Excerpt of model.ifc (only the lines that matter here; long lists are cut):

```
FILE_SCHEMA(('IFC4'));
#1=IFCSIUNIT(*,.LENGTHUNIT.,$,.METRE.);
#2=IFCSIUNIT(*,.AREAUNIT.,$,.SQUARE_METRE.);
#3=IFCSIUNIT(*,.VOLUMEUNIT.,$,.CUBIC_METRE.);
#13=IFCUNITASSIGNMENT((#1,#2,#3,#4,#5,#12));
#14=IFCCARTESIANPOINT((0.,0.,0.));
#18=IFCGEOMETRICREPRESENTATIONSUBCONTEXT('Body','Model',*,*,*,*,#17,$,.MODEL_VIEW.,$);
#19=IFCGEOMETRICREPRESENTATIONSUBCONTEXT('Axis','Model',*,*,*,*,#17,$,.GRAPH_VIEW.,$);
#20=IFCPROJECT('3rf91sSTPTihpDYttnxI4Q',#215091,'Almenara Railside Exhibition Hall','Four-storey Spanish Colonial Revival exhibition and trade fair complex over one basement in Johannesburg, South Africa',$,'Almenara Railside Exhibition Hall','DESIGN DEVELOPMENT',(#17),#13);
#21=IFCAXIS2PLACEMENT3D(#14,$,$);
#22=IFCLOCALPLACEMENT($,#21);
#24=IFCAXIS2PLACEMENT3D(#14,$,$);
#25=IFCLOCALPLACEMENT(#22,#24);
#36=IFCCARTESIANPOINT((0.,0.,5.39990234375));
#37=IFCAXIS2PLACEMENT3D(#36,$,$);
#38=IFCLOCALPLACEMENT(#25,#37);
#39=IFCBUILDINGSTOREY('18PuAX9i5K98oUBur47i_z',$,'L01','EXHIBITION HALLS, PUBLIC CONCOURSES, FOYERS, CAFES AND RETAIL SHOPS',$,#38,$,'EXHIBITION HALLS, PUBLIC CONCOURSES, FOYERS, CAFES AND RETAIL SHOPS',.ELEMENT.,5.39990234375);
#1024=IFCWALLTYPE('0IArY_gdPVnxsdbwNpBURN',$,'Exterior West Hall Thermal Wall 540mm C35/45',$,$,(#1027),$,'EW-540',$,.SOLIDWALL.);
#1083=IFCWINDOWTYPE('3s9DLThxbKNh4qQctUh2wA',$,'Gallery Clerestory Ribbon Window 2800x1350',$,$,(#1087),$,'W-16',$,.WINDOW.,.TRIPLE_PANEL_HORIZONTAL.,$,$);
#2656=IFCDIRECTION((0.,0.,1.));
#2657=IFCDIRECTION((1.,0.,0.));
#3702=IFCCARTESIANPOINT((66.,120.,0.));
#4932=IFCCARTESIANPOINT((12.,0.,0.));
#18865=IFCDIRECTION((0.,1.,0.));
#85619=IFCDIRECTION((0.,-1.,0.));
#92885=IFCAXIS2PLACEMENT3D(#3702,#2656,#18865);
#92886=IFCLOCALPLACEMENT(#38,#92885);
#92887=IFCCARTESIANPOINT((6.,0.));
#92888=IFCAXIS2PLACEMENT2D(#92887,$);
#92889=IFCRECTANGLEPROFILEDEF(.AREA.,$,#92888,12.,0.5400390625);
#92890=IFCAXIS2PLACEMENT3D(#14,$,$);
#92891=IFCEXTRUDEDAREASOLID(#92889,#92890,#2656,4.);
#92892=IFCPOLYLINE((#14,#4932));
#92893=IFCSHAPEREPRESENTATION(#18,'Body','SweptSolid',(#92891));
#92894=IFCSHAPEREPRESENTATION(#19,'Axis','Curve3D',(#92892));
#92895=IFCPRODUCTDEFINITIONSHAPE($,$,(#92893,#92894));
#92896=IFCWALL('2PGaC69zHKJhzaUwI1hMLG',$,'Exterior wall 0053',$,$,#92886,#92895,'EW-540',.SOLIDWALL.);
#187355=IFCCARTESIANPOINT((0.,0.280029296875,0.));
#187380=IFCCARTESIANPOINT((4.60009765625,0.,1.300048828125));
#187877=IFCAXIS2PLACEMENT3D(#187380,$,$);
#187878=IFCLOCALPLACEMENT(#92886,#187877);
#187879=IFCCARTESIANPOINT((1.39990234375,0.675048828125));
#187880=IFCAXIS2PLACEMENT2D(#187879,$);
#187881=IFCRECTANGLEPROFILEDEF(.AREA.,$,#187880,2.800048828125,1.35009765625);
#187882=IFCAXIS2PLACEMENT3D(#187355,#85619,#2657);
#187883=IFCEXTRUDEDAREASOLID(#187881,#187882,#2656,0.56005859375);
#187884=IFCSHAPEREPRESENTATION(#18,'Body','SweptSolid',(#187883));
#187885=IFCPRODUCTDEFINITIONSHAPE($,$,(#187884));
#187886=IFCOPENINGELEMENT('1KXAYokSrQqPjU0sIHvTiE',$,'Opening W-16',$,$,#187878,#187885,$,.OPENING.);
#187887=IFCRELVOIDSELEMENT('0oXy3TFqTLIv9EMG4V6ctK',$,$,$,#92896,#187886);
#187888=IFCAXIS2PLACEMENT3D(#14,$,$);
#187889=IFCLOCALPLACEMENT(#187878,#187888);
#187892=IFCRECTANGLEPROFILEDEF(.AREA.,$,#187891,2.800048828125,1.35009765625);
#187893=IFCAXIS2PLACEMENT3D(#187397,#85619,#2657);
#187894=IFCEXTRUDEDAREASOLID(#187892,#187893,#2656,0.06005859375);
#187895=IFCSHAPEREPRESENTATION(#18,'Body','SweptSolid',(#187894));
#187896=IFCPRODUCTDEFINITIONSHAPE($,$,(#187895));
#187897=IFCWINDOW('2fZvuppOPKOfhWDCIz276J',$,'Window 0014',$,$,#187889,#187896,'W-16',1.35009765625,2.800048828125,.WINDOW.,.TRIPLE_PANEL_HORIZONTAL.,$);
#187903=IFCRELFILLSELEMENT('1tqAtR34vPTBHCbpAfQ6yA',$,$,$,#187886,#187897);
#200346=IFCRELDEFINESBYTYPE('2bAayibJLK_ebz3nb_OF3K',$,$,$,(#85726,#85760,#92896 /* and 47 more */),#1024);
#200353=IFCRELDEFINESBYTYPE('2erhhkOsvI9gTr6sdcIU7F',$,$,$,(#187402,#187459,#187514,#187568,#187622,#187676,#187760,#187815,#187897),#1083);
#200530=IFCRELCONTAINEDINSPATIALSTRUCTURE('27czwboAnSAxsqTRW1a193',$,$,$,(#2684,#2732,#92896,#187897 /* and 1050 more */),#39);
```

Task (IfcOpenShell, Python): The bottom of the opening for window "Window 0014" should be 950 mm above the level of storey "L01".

```python
import numpy as np
import ifcopenshell
import ifcopenshell.api.geometry
import ifcopenshell.geom
import ifcopenshell.util.element
import ifcopenshell.util.placement
import ifcopenshell.util.shape
import ifcopenshell.util.unit

model = ifcopenshell.open("model.ifc")
unit_scale = ifcopenshell.util.unit.calculate_unit_scale(model)

window = model.by_guid("2fZvuppOPKOfhWDCIz276J")
opening = window.FillsVoids[0].RelatingOpeningElement
storey = ifcopenshell.util.element.get_container(window, ifc_class="IfcBuildingStorey")
level = ifcopenshell.util.placement.get_local_placement(storey.ObjectPlacement)[2, 3]

# The opening's origin need not be at the sill, so measure its lowest point.
shape = ifcopenshell.geom.create_shape(ifcopenshell.geom.settings(), opening)
bottom = ifcopenshell.util.shape.get_shape_bottom_elevation(shape, shape.geometry) / unit_scale
dz = level + 0.95 / unit_scale - bottom

shift = np.array([0.0, 0.0, dz])
# The window is placed relative to its opening, so it follows when the opening moves.
matrix = ifcopenshell.util.placement.get_local_placement(opening.ObjectPlacement)
matrix[:3, 3] += shift
ifcopenshell.api.geometry.edit_object_placement(
    model, product=opening, matrix=matrix, is_si=False, should_transform_children=True
)

print(f"moved by {dz * unit_scale:+.3f} m")

model.write("model-out.ifc")
```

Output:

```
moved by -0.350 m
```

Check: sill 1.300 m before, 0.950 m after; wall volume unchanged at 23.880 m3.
